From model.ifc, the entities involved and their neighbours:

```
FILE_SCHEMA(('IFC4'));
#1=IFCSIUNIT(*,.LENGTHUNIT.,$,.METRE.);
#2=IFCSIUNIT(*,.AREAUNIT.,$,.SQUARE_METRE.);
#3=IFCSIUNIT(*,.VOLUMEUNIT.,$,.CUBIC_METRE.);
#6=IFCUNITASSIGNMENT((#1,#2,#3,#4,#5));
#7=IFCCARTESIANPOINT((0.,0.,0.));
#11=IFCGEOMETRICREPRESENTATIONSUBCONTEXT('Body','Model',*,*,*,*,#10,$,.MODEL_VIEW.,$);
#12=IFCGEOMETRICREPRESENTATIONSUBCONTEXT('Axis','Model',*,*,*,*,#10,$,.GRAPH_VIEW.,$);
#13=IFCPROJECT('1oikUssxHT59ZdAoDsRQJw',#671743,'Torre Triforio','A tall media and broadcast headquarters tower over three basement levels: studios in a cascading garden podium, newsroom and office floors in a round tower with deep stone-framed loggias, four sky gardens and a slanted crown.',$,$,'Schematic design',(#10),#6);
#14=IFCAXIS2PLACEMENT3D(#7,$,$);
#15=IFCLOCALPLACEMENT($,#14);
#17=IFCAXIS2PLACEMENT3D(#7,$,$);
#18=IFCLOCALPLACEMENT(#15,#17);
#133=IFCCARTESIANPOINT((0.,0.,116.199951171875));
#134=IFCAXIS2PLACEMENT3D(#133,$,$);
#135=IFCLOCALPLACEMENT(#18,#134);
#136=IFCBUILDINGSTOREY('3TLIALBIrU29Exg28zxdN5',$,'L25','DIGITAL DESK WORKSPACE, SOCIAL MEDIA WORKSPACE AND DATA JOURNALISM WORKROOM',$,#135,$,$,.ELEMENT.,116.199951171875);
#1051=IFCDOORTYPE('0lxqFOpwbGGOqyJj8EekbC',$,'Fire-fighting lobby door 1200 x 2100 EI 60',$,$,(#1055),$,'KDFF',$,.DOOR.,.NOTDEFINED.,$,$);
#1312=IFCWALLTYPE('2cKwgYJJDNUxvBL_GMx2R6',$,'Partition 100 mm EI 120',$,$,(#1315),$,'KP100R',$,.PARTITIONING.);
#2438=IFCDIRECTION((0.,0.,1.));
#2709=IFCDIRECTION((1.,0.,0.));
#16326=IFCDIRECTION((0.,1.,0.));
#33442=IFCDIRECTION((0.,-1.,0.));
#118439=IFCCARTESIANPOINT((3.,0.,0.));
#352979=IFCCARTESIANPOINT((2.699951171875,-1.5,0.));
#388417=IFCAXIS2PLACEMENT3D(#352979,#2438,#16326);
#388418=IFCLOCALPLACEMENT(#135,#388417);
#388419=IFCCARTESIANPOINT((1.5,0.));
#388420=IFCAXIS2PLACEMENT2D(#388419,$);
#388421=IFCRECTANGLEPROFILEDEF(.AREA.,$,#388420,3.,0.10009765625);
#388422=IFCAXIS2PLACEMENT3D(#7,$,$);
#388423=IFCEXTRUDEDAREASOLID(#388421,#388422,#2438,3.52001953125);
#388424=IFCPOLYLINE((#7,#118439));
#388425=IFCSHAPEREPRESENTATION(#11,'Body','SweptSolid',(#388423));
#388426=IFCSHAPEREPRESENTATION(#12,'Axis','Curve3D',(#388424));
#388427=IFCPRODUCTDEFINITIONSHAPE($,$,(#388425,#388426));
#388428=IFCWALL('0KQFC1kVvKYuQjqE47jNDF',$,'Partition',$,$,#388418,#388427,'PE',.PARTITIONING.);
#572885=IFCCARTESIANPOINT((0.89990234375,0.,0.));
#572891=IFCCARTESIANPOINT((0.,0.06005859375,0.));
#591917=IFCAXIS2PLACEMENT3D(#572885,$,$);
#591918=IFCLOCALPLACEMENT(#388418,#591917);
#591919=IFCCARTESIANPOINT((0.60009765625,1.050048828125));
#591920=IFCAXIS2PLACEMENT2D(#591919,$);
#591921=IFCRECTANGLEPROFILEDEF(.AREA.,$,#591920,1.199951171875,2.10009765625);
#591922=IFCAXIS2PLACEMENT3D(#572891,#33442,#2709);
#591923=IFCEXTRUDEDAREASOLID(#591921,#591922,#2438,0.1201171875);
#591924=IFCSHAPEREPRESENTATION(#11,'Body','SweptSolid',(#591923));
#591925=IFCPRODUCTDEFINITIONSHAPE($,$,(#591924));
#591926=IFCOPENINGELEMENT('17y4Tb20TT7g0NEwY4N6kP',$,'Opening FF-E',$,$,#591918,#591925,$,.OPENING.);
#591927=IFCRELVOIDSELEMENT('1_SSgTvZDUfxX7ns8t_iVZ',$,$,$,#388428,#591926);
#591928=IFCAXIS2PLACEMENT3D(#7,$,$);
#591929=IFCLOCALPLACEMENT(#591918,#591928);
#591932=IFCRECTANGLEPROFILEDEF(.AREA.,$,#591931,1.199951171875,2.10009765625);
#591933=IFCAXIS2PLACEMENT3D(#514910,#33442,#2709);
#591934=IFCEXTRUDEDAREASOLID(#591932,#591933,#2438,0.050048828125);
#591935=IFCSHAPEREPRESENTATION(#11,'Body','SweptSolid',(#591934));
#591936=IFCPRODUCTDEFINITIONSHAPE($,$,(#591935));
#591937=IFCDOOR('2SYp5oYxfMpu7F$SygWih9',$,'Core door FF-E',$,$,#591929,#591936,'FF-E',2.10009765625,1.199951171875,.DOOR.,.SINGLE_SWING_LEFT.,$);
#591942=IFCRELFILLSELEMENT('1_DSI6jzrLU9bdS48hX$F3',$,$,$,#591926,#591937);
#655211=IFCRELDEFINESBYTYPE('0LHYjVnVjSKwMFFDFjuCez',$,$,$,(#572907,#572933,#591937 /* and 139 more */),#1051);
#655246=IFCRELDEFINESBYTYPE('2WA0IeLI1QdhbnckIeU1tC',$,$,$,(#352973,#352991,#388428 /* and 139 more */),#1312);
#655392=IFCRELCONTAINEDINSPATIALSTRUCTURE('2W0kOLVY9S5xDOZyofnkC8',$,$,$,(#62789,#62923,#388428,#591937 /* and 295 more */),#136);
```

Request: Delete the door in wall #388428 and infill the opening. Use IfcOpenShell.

```python
import ifcopenshell
import ifcopenshell.api.feature
import ifcopenshell.api.root
import ifcopenshell.geom
import ifcopenshell.util.shape

model = ifcopenshell.open("model.ifc")
settings = ifcopenshell.geom.settings()


def volume(element):
    """Net volume in cubic metres, openings subtracted."""
    shape = ifcopenshell.geom.create_shape(settings, element)
    return ifcopenshell.util.shape.get_volume(shape.geometry)


door = model.by_guid("2SYp5oYxfMpu7F$SygWih9")
opening = door.FillsVoids[0].RelatingOpeningElement
wall = opening.VoidsElements[0].RelatingBuildingElement
before = volume(wall)

ifcopenshell.api.root.remove_product(model, product=door)
ifcopenshell.api.feature.remove_feature(model, feature=opening)

after = volume(wall)

print(f"wall volume {before:.3f} -> {after:.3f} m3")

model.write("model_v2.ifc")
```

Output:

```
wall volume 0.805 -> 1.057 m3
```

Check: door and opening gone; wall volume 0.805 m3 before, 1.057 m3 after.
